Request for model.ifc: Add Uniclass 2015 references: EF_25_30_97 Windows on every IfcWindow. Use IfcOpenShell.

First a look at what the model holds.

```python
import ifcopenshell

model = ifcopenshell.open("model.ifc")
print(model.schema)
print("classifications:", [c.Name for c in model.by_type("IfcClassification")])
for ifc_class in ("IfcDoor", "IfcRoof", "IfcStair", "IfcWall", "IfcWindow"):
    print(ifc_class, len(model.by_type(ifc_class)))
```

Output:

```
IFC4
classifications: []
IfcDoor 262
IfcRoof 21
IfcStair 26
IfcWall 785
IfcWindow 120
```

```python
import ifcopenshell
import ifcopenshell.api.classification

model = ifcopenshell.open("model.ifc")

system = ifcopenshell.api.classification.add_classification(model, classification="Uniclass 2015")

codes = {
    "IfcWindow": ("EF_25_30_97", "Windows"),
}
for ifc_class, (code, name) in codes.items():
    products = model.by_type(ifc_class)
    ifcopenshell.api.classification.add_reference(
        model, products=products, classification=system, identification=code, name=name
    )
    print(code, len(products))

model.write("model_v2.ifc")
```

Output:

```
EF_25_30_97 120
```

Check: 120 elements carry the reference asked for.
